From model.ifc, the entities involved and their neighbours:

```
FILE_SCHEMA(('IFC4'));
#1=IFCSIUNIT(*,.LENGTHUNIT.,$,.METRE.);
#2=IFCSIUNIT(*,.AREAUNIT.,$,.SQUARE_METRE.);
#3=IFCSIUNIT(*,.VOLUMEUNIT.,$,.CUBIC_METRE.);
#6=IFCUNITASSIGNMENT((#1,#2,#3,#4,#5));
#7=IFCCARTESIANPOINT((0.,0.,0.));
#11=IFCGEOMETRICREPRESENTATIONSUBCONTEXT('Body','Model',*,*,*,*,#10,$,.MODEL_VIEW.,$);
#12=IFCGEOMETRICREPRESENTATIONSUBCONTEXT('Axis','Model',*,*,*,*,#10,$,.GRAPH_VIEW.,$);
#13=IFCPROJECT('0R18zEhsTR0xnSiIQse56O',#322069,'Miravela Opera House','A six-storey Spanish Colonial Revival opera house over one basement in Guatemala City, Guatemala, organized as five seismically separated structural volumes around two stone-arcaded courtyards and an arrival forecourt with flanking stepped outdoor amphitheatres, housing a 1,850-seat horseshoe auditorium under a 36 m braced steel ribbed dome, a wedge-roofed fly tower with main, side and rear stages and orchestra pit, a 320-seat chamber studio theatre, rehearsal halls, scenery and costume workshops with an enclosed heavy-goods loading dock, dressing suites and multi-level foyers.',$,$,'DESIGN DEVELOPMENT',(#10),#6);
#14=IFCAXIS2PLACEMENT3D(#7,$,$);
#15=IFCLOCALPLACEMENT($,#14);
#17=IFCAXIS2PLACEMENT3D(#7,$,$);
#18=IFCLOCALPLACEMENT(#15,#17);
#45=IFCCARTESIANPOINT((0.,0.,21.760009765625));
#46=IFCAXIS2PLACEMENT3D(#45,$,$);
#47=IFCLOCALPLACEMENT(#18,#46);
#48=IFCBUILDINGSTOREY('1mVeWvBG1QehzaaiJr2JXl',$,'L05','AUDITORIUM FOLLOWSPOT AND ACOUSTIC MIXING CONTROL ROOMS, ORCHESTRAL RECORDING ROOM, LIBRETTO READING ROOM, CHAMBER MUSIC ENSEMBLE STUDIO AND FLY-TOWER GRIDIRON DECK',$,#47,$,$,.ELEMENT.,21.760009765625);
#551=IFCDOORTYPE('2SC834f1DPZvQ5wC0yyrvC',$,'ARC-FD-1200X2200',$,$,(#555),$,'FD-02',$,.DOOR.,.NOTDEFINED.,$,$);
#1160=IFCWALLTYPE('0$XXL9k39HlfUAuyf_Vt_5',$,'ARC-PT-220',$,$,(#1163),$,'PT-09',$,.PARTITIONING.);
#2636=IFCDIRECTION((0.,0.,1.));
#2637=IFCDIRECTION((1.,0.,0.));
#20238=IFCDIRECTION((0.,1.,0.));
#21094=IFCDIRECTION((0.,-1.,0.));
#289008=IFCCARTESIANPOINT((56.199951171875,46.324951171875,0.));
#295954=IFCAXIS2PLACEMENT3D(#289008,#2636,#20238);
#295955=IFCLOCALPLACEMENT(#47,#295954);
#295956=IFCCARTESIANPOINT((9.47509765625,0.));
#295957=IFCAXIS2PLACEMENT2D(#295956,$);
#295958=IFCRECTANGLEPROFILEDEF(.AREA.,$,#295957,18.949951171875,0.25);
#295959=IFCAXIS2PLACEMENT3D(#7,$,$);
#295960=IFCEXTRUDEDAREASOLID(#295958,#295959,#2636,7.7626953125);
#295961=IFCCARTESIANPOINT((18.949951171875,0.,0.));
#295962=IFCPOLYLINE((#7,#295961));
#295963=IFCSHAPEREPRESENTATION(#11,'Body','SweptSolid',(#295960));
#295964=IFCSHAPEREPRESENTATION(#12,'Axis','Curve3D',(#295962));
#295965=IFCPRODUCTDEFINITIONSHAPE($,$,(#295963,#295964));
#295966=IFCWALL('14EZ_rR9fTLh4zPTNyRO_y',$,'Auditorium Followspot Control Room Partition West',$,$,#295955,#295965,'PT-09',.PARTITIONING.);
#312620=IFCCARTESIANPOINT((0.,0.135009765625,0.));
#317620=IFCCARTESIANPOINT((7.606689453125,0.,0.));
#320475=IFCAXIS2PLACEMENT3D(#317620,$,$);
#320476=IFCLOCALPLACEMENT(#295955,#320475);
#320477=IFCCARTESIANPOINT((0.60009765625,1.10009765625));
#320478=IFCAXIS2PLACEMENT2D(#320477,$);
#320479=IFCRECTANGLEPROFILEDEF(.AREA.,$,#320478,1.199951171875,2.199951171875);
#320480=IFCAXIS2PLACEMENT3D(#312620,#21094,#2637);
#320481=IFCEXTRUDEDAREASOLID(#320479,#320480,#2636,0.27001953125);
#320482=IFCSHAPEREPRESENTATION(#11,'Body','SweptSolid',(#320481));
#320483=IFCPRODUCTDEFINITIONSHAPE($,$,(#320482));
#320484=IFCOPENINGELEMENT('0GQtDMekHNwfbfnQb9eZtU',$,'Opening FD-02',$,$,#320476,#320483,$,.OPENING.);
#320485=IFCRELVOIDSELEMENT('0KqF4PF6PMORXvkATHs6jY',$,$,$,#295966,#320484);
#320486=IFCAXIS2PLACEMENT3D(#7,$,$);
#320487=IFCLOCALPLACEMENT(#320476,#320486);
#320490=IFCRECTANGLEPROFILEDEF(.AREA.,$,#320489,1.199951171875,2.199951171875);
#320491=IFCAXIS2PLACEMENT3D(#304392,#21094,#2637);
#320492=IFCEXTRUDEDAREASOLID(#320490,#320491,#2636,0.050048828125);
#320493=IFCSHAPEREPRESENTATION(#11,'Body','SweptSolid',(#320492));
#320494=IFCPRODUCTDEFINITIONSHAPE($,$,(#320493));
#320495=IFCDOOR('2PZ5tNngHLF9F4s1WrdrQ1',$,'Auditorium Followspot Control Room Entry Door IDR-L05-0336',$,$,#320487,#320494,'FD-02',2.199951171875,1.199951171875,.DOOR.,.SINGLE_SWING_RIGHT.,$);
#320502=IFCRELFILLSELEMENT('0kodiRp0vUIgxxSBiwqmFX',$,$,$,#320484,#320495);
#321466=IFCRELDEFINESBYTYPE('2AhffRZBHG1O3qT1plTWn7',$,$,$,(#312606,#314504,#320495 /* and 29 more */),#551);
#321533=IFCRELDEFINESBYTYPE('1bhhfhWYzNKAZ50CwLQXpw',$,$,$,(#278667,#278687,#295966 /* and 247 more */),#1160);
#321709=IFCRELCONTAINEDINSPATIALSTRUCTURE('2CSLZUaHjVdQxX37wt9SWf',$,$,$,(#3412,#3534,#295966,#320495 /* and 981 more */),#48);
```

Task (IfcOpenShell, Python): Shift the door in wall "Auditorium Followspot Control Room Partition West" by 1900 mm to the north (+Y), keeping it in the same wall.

```python
import ifcopenshell
import ifcopenshell.api.geometry
import ifcopenshell.util.placement
import ifcopenshell.util.unit

model = ifcopenshell.open("model.ifc")
unit_scale = ifcopenshell.util.unit.calculate_unit_scale(model)

door = model.by_guid("2PZ5tNngHLF9F4s1WrdrQ1")
opening = door.FillsVoids[0].RelatingOpeningElement
wall = opening.VoidsElements[0].RelatingBuildingElement

wall_matrix = ifcopenshell.util.placement.get_local_placement(wall.ObjectPlacement)
shift = wall_matrix[:3, 0] * 1.9 / unit_scale
before = ifcopenshell.util.placement.get_local_placement(door.ObjectPlacement)[:3, 3].copy()

# The door is placed relative to its opening, so it follows when the opening moves.
matrix = ifcopenshell.util.placement.get_local_placement(opening.ObjectPlacement)
matrix[:3, 3] += shift
ifcopenshell.api.geometry.edit_object_placement(
    model, product=opening, matrix=matrix, is_si=False, should_transform_children=True
)

after = ifcopenshell.util.placement.get_local_placement(door.ObjectPlacement)[:3, 3]
print("door moved by", (after - before).round(3) + 0.0)

model.write("model_updated.ifc")
```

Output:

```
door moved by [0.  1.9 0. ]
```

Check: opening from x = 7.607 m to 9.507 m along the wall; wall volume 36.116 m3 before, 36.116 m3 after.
